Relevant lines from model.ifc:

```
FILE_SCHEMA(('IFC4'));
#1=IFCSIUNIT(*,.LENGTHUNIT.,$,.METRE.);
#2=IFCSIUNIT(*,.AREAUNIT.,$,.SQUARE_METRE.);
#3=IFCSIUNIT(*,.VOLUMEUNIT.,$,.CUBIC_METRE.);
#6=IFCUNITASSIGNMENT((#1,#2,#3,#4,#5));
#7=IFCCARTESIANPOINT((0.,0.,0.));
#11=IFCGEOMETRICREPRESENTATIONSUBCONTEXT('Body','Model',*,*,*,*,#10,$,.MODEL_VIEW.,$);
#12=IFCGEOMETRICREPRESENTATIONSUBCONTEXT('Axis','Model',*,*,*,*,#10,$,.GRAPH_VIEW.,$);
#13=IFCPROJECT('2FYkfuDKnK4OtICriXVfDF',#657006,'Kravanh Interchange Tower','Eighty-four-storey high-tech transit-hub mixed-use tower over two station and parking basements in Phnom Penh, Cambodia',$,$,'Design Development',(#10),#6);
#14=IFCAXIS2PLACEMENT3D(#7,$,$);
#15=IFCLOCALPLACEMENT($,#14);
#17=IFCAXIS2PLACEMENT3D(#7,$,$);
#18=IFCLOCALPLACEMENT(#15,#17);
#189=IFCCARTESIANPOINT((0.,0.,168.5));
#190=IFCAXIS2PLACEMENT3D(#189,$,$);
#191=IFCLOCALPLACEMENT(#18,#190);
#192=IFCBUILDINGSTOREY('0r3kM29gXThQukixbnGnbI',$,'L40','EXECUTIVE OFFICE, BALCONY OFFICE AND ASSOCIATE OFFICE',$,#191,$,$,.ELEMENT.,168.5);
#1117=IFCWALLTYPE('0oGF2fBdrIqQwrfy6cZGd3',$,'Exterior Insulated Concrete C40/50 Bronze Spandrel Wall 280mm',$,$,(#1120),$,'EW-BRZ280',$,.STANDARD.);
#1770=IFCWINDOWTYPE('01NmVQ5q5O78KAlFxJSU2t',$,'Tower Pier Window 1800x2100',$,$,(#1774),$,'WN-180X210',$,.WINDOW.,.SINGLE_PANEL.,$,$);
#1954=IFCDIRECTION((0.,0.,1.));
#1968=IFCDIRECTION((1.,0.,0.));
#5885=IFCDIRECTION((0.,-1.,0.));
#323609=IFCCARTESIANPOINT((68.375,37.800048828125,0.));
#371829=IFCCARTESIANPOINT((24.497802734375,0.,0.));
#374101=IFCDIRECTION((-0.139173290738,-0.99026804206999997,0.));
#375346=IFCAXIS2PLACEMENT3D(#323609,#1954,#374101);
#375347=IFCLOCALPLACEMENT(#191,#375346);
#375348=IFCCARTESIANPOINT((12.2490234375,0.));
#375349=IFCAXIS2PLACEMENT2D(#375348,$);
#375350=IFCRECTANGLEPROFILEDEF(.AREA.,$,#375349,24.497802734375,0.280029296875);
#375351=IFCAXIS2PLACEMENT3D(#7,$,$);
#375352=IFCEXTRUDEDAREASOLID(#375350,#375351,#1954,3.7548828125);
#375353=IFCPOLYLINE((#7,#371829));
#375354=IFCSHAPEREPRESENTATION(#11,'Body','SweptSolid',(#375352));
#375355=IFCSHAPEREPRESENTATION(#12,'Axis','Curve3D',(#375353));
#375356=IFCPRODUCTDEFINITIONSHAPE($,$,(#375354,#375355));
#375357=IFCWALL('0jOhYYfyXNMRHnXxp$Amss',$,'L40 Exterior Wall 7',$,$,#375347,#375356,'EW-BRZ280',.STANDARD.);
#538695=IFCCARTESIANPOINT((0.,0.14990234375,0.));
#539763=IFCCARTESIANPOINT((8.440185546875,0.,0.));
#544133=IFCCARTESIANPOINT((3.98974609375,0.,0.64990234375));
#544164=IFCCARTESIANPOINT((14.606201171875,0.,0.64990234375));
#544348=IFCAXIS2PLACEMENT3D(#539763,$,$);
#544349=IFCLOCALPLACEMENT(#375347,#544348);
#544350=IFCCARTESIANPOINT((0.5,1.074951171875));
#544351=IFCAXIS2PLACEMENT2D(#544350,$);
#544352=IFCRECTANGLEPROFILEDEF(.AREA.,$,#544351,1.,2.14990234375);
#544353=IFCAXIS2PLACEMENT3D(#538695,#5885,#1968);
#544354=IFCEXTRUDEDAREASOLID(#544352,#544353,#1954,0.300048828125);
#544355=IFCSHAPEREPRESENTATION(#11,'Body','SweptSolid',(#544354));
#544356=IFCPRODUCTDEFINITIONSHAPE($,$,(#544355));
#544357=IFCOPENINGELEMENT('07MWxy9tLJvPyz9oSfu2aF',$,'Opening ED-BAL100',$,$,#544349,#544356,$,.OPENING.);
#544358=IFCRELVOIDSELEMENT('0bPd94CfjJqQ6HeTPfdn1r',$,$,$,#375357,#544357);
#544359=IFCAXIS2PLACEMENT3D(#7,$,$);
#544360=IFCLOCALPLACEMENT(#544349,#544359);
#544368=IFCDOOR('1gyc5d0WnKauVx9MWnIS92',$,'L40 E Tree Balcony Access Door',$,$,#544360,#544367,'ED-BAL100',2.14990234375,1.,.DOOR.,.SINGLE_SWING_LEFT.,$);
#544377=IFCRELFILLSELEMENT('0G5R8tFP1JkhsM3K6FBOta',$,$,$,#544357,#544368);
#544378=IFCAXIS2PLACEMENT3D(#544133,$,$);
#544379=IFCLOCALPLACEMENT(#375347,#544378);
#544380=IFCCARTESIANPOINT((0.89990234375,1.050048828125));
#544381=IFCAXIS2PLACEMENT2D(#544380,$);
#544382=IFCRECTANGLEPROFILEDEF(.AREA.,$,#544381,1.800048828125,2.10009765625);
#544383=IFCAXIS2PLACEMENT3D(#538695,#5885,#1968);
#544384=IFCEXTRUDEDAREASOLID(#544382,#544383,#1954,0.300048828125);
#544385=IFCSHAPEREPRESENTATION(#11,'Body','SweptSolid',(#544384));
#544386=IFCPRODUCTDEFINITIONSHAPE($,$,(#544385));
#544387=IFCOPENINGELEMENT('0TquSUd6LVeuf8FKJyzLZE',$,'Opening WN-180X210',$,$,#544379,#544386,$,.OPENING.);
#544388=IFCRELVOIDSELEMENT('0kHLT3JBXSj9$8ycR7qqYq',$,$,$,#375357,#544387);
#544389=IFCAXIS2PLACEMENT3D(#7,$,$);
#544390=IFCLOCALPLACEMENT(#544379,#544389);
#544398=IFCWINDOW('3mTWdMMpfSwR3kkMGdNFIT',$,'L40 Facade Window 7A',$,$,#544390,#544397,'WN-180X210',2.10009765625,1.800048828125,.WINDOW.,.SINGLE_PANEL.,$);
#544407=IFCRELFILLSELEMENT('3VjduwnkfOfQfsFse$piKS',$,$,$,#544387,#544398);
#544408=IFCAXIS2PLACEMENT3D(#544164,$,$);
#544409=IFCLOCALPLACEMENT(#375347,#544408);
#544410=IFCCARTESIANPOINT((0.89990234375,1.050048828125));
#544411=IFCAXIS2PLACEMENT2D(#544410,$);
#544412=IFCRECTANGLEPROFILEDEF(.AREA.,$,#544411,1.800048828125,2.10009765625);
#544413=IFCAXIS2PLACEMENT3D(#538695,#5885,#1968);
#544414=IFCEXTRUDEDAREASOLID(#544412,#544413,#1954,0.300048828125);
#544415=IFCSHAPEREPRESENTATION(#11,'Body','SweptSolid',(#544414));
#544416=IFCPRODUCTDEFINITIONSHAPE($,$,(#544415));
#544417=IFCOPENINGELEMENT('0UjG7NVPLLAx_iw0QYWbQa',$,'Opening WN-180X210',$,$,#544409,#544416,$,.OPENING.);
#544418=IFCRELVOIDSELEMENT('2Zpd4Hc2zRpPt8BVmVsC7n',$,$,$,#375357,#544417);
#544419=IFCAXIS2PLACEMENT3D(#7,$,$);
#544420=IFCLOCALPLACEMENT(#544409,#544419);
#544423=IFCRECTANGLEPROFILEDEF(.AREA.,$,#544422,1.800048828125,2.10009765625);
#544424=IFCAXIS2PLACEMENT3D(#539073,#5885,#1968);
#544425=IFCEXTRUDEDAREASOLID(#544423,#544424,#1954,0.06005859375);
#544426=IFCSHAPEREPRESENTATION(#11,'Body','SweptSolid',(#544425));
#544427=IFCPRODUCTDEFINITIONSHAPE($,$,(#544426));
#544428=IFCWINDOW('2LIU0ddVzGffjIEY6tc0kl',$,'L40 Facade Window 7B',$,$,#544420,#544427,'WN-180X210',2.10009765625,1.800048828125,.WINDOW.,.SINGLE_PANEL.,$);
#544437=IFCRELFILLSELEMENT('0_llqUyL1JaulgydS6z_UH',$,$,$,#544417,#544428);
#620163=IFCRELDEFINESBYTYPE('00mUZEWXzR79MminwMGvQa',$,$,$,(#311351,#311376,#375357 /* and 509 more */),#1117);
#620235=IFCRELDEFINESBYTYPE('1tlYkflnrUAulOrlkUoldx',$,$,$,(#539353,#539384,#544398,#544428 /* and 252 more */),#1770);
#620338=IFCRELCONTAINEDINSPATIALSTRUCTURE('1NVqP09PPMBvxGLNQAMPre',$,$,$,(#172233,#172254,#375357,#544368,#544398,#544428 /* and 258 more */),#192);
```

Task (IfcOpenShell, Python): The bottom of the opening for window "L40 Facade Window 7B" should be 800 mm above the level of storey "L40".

```python
import numpy as np
import ifcopenshell
import ifcopenshell.api.geometry
import ifcopenshell.geom
import ifcopenshell.util.element
import ifcopenshell.util.placement
import ifcopenshell.util.shape
import ifcopenshell.util.unit

model = ifcopenshell.open("model.ifc")
unit_scale = ifcopenshell.util.unit.calculate_unit_scale(model)

window = model.by_guid("2LIU0ddVzGffjIEY6tc0kl")
opening = window.FillsVoids[0].RelatingOpeningElement
storey = ifcopenshell.util.element.get_container(window, ifc_class="IfcBuildingStorey")
level = ifcopenshell.util.placement.get_local_placement(storey.ObjectPlacement)[2, 3]

# The opening's origin need not be at the sill, so measure its lowest point.
shape = ifcopenshell.geom.create_shape(ifcopenshell.geom.settings(), opening)
bottom = ifcopenshell.util.shape.get_shape_bottom_elevation(shape, shape.geometry) / unit_scale
dz = level + 0.8 / unit_scale - bottom

shift = np.array([0.0, 0.0, dz])
# The window is placed relative to its opening, so it follows when the opening moves.
matrix = ifcopenshell.util.placement.get_local_placement(opening.ObjectPlacement)
matrix[:3, 3] += shift
ifcopenshell.api.geometry.edit_object_placement(
    model, product=opening, matrix=matrix, is_si=False, should_transform_children=True
)

print(f"moved by {dz * unit_scale:+.3f} m")

model.write("model_edited.ifc")
```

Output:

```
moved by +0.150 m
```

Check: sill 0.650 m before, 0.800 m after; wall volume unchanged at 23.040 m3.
